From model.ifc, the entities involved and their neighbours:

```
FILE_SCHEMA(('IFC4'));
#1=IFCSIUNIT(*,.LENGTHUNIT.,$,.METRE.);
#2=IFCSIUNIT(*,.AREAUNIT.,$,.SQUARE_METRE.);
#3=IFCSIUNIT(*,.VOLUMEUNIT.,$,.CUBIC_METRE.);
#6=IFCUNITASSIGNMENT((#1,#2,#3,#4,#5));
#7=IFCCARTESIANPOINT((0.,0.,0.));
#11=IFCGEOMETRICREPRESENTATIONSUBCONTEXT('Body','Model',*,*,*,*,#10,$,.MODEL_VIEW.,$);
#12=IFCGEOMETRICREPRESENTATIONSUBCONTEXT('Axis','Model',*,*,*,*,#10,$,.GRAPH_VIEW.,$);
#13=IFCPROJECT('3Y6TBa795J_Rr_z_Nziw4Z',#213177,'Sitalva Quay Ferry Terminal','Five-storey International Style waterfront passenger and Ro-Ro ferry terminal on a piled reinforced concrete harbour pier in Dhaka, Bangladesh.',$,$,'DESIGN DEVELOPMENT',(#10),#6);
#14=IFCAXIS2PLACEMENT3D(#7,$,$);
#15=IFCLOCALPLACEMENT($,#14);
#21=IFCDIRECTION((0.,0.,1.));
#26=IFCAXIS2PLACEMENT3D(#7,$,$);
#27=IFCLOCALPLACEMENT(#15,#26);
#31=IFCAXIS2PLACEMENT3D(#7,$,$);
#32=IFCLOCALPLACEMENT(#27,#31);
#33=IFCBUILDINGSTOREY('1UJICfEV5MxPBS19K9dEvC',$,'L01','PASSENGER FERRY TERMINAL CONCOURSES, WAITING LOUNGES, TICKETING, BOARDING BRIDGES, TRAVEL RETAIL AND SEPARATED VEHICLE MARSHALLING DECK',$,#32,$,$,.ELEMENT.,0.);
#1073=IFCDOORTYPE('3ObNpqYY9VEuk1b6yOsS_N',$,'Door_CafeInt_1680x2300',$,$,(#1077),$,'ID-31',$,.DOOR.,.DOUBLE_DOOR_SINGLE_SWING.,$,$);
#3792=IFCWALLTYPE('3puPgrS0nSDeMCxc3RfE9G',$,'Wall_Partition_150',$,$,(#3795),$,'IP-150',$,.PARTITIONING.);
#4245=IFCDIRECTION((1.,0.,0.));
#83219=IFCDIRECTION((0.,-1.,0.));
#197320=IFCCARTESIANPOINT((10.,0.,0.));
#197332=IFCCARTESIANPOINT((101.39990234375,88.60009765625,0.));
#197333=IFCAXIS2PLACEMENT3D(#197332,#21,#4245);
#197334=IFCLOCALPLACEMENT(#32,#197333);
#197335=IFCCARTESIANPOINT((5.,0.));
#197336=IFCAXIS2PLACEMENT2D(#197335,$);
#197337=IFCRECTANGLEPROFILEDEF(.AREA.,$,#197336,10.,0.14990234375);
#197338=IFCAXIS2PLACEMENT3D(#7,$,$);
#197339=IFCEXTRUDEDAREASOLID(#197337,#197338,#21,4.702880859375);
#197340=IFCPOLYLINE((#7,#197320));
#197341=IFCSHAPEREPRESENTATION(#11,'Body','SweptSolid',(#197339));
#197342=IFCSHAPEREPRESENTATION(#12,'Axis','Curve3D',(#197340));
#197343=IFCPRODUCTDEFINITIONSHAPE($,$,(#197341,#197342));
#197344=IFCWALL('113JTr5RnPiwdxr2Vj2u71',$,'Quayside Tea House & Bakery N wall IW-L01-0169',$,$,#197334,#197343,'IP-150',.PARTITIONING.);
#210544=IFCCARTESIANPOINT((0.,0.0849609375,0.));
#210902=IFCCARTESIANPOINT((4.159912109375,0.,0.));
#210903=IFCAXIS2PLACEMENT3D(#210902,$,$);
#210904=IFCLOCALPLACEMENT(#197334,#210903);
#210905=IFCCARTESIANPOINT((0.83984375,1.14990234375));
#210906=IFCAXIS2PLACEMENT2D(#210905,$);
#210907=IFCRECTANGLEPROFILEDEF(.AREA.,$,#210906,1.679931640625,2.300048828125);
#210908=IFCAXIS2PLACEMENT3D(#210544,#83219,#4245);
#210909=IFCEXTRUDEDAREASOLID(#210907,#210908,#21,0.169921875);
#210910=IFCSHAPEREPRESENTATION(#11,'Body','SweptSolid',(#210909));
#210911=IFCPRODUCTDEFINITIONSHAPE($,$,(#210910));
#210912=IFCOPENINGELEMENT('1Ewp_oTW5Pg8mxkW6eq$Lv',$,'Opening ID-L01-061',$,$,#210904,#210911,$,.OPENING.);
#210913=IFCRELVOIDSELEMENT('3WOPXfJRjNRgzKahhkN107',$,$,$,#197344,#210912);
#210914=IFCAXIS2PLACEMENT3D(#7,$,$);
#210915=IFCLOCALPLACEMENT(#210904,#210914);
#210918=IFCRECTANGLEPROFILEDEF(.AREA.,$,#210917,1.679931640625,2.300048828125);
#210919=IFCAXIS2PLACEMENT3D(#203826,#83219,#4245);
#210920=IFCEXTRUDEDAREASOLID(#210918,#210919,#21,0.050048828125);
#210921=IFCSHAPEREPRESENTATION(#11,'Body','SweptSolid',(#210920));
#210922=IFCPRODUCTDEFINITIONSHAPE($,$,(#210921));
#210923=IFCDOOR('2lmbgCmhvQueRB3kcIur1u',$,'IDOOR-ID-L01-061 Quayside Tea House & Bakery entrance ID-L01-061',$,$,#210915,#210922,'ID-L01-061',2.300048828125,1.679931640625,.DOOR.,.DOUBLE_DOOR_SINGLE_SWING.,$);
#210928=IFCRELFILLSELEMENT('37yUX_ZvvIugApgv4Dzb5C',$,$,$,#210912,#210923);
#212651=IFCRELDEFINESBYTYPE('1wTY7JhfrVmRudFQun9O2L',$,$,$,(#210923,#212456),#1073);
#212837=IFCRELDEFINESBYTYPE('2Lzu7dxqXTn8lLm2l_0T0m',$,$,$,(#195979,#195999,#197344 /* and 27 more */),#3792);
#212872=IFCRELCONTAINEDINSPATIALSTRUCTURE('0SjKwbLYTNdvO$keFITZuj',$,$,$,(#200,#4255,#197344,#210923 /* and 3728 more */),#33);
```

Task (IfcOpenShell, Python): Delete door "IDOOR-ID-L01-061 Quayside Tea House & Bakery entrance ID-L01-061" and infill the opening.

```python
import ifcopenshell
import ifcopenshell.api.feature
import ifcopenshell.api.root
import ifcopenshell.geom
import ifcopenshell.util.shape

model = ifcopenshell.open("model.ifc")
settings = ifcopenshell.geom.settings()


def volume(element):
    """Net volume in cubic metres, openings subtracted."""
    shape = ifcopenshell.geom.create_shape(settings, element)
    return ifcopenshell.util.shape.get_volume(shape.geometry)


door = model.by_guid("2lmbgCmhvQueRB3kcIur1u")
opening = door.FillsVoids[0].RelatingOpeningElement
wall = opening.VoidsElements[0].RelatingBuildingElement
before = volume(wall)

ifcopenshell.api.root.remove_product(model, product=door)
ifcopenshell.api.feature.remove_feature(model, feature=opening)

after = volume(wall)

print(f"wall volume {before:.3f} -> {after:.3f} m3")

model.write("model-out.ifc")
```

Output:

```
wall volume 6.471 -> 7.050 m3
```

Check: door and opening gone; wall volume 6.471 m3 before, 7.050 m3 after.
